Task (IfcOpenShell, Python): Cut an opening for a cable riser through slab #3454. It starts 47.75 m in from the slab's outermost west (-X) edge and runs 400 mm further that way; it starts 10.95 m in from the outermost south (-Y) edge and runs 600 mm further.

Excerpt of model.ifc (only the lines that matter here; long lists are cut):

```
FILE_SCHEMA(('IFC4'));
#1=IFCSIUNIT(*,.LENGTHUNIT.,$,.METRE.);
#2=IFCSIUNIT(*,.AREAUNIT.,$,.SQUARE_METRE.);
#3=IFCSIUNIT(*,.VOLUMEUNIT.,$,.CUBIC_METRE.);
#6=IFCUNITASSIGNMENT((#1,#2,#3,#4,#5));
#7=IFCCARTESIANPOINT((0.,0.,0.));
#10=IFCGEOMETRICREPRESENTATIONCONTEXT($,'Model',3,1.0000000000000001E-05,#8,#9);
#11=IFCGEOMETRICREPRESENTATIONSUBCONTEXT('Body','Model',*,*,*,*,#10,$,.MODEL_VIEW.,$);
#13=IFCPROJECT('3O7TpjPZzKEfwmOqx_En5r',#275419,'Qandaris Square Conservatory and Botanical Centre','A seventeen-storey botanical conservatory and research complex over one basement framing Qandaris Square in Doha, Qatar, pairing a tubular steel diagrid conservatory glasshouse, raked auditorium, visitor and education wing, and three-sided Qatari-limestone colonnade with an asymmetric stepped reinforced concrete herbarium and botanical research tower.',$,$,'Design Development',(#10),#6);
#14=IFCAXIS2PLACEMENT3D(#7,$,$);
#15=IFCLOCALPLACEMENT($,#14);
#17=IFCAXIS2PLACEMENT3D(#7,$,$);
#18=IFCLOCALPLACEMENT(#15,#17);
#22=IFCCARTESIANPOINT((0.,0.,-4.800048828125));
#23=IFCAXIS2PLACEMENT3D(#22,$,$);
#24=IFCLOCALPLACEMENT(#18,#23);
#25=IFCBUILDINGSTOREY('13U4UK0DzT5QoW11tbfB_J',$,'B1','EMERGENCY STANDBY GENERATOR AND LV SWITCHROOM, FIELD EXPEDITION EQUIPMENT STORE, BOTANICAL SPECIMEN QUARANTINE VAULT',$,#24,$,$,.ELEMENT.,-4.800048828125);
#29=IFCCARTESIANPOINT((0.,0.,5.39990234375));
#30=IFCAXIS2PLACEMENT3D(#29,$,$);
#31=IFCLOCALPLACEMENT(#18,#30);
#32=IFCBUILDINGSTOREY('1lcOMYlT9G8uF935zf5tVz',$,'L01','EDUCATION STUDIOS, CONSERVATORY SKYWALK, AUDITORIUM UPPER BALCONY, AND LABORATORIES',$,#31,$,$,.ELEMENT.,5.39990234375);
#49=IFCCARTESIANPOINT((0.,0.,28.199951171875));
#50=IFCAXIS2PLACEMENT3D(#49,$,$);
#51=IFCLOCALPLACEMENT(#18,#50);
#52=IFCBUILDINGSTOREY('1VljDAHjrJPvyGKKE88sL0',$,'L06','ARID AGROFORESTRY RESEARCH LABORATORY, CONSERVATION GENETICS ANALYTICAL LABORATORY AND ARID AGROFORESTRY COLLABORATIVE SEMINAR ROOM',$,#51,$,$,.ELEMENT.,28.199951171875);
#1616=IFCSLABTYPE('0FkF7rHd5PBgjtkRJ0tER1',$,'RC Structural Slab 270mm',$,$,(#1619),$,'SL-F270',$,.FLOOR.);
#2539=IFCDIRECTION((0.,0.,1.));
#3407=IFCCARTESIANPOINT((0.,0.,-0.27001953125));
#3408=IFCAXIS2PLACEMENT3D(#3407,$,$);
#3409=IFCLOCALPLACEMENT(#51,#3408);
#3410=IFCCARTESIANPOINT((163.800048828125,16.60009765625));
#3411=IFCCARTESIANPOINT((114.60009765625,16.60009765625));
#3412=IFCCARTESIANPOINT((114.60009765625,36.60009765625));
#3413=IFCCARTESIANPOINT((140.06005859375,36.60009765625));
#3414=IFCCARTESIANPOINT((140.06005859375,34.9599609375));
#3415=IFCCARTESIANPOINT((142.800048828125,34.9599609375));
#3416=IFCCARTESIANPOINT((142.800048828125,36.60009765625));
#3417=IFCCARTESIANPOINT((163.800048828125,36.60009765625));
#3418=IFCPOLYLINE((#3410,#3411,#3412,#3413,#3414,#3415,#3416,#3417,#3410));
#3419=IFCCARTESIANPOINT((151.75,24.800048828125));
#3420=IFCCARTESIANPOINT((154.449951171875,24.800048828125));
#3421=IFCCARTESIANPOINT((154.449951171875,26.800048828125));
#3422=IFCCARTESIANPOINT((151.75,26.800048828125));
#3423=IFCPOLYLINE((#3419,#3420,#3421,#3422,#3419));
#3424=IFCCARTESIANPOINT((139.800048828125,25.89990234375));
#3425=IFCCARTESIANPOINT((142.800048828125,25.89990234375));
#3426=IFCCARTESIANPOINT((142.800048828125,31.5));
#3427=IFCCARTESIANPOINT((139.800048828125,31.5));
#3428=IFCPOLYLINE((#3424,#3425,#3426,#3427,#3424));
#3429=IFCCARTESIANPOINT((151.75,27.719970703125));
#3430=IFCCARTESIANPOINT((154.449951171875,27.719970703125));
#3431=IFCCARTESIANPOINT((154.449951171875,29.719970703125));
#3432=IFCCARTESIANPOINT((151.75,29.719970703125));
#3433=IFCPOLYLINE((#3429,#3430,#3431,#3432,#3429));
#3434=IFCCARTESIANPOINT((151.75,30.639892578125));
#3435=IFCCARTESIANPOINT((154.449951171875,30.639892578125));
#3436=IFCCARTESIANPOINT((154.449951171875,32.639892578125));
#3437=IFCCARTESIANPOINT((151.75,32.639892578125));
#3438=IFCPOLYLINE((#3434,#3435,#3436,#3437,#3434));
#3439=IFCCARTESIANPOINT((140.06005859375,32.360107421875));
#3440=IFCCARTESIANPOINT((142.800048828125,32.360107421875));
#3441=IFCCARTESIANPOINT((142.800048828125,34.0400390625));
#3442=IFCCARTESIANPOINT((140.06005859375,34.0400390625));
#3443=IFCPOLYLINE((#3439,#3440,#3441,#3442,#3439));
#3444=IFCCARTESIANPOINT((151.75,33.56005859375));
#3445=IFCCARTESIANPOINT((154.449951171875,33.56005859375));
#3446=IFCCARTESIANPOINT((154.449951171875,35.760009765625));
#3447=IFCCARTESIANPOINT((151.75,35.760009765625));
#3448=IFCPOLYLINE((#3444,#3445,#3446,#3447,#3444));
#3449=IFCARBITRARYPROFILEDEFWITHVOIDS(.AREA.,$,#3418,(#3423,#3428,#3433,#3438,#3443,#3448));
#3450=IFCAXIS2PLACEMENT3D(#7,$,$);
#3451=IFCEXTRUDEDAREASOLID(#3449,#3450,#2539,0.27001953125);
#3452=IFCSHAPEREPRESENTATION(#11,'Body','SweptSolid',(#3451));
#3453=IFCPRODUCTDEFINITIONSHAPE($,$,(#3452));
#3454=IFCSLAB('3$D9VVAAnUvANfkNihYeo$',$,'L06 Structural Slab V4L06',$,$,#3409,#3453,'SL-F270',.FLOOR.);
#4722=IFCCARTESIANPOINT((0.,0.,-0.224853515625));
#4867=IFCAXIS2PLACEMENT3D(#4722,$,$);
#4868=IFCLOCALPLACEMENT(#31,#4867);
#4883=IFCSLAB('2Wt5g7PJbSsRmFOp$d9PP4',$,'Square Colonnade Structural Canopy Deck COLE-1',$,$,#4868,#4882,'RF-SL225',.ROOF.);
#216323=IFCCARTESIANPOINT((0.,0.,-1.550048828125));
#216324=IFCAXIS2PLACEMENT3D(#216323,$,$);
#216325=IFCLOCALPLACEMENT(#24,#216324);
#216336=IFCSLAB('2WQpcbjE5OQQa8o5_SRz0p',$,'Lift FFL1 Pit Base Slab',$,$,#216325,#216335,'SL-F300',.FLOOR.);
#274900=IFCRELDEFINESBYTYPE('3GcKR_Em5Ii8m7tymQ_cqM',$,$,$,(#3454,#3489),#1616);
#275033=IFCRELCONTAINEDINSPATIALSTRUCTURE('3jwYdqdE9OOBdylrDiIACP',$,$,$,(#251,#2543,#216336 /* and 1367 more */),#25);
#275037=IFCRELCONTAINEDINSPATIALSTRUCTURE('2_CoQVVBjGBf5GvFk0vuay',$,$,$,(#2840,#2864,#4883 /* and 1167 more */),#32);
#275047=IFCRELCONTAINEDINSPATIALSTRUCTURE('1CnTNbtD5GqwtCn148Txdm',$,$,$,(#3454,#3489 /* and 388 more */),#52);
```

```python
import numpy as np
import ifcopenshell
import ifcopenshell.api.feature
import ifcopenshell.api.geometry
import ifcopenshell.api.root
import ifcopenshell.geom
import ifcopenshell.util.placement
import ifcopenshell.util.representation
import ifcopenshell.util.shape
import ifcopenshell.util.unit

model = ifcopenshell.open("model.ifc")
unit_scale = ifcopenshell.util.unit.calculate_unit_scale(model)
settings = ifcopenshell.geom.settings()


def volume(element):
    """Net volume in cubic metres, openings subtracted."""
    shape = ifcopenshell.geom.create_shape(settings, element)
    return ifcopenshell.util.shape.get_volume(shape.geometry)


slab = model.by_id(3454)
before = volume(slab)

# Extent in the slab's own axes, in metres. The edges named are its -X and -Y sides.
slab_shape = ifcopenshell.geom.create_shape(settings, slab)
vertices = ifcopenshell.util.shape.get_vertices(slab_shape.geometry)
x_min, y_min, bottom = vertices.min(axis=0)
top = vertices[:, 2].max()

opening = ifcopenshell.api.root.create_entity(model, ifc_class="IfcOpeningElement", name="Cable riser opening", predefined_type="OPENING")
context = ifcopenshell.util.representation.get_context(model, "Model", "Body", "MODEL_VIEW")
width, depth = 0.4, 0.6
outline = [(0.0, 0.0), (width, 0.0), (width, depth), (0.0, depth), (0.0, 0.0)]
# Overshoot both faces by 50 mm so the cut is clean.
shape = ifcopenshell.api.geometry.add_slab_representation(
    model, context=context, depth=top - bottom + 0.1, polyline=outline
)
ifcopenshell.api.geometry.assign_representation(model, product=opening, representation=shape)

matrix = ifcopenshell.util.placement.get_local_placement(slab.ObjectPlacement)
matrix[:, 3] = matrix @ np.append(np.array([x_min + 47.75, y_min + 10.95, bottom - 0.05]) / unit_scale, 1.0)
ifcopenshell.api.geometry.edit_object_placement(model, product=opening, matrix=matrix, is_si=False)
ifcopenshell.api.feature.add_feature(model, feature=opening, element=slab)

after = volume(slab)

print(f"slab volume {before:.3f} -> {after:.3f} m3")

model.write("model_updated.ifc")
```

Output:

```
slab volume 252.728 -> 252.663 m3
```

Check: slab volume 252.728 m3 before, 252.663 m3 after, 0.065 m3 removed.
